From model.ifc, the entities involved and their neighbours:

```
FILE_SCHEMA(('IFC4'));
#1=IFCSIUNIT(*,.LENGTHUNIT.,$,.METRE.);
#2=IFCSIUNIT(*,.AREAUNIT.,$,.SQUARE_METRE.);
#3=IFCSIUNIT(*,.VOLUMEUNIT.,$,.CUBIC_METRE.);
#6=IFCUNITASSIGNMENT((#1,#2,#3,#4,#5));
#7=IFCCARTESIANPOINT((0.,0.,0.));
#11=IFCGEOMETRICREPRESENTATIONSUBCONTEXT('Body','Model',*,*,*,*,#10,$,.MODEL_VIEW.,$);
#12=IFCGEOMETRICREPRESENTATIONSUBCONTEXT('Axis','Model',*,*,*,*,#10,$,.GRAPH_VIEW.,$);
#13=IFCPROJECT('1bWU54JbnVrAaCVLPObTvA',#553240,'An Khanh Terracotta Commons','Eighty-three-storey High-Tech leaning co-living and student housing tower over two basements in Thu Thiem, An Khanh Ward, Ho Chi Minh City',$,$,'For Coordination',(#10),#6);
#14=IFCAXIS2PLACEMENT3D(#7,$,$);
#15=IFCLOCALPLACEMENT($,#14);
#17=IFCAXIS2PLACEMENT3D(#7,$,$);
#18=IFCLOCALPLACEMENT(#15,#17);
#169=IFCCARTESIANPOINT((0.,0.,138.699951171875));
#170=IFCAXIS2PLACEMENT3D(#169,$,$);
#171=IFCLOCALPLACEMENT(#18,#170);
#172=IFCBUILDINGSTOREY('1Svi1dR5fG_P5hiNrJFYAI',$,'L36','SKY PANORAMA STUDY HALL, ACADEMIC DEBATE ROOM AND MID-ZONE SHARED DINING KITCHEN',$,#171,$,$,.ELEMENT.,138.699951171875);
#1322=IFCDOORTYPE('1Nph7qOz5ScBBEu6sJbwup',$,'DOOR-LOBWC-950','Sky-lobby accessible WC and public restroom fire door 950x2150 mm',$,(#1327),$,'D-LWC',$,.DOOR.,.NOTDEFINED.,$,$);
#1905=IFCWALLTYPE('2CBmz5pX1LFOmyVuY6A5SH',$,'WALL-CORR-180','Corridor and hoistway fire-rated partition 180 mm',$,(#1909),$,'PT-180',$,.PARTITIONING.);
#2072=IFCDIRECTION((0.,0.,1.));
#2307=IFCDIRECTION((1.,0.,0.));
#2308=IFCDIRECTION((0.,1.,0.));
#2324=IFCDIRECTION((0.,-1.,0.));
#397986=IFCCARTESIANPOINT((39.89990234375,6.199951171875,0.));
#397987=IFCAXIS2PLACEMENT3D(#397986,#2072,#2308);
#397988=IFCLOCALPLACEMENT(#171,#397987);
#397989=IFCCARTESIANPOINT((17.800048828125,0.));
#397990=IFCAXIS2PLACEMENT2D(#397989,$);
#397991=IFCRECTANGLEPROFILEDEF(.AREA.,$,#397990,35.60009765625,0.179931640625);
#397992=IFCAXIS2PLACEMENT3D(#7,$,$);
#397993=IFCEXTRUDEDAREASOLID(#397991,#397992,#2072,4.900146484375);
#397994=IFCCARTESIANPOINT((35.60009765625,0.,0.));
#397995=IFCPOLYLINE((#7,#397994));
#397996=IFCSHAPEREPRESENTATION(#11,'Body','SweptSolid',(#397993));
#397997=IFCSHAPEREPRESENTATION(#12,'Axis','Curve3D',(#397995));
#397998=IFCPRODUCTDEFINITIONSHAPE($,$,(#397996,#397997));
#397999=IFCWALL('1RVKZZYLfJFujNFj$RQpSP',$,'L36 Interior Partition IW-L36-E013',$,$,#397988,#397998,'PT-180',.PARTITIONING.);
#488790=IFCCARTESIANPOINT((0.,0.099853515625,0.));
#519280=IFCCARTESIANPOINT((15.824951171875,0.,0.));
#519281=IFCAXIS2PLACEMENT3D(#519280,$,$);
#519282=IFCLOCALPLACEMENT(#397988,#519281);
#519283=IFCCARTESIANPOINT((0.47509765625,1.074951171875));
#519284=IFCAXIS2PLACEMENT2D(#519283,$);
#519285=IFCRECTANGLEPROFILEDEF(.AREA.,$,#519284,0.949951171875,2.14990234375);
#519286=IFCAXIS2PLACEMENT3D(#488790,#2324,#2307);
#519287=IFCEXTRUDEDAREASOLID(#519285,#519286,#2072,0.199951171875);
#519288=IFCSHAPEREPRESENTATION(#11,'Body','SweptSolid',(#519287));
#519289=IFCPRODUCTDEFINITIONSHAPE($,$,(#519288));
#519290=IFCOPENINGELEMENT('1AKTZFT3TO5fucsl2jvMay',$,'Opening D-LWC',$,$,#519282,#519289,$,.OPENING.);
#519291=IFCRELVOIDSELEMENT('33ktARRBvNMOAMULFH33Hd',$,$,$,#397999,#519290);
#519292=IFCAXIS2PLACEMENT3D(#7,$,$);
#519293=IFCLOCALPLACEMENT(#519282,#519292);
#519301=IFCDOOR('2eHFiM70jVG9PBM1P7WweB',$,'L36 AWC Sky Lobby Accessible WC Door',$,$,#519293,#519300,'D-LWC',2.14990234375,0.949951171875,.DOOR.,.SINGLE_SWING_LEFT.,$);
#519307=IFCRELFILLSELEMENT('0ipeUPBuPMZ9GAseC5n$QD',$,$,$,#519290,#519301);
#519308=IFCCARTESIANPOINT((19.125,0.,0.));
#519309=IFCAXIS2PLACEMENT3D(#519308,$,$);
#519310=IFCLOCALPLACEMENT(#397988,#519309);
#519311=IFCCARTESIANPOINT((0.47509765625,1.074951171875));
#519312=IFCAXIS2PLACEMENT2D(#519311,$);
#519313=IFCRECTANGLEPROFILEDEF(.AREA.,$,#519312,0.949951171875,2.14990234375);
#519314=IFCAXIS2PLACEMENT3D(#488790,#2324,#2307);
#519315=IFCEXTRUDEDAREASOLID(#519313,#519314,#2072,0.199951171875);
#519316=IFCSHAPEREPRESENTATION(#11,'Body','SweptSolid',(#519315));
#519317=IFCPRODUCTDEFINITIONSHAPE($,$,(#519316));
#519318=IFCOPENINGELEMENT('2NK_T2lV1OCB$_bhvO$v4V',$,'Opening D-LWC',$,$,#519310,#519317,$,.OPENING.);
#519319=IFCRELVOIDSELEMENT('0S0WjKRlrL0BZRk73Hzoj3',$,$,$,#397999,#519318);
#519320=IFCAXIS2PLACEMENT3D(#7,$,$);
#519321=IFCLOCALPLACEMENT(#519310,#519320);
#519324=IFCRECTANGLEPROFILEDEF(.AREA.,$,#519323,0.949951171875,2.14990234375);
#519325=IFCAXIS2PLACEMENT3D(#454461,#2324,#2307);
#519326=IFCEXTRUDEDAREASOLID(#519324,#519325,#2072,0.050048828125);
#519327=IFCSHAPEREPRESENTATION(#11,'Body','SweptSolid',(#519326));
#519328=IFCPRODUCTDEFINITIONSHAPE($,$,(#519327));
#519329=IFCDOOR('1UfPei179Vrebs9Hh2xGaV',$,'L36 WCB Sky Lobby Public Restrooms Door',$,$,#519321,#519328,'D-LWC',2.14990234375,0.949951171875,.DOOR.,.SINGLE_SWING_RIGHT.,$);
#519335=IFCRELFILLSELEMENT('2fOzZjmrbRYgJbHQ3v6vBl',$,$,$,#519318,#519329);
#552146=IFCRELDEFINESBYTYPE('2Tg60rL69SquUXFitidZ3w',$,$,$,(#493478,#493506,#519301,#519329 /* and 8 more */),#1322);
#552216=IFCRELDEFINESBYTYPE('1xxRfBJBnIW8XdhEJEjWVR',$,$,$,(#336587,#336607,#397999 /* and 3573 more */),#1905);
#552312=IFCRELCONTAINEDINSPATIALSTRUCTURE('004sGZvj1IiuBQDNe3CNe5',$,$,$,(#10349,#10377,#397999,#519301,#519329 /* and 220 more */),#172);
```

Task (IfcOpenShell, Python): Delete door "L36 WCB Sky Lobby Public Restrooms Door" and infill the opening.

```python
import ifcopenshell
import ifcopenshell.api.feature
import ifcopenshell.api.root
import ifcopenshell.geom
import ifcopenshell.util.shape

model = ifcopenshell.open("model.ifc")
settings = ifcopenshell.geom.settings()


def volume(element):
    """Net volume in cubic metres, openings subtracted."""
    shape = ifcopenshell.geom.create_shape(settings, element)
    return ifcopenshell.util.shape.get_volume(shape.geometry)


door = model.by_guid("1UfPei179Vrebs9Hh2xGaV")
opening = door.FillsVoids[0].RelatingOpeningElement
wall = opening.VoidsElements[0].RelatingBuildingElement
before = volume(wall)

ifcopenshell.api.root.remove_product(model, product=door)
ifcopenshell.api.feature.remove_feature(model, feature=opening)

after = volume(wall)

print(f"wall volume {before:.3f} -> {after:.3f} m3")

model.write("model-out.ifc")
```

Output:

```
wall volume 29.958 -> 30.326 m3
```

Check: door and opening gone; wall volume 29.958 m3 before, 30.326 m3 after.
